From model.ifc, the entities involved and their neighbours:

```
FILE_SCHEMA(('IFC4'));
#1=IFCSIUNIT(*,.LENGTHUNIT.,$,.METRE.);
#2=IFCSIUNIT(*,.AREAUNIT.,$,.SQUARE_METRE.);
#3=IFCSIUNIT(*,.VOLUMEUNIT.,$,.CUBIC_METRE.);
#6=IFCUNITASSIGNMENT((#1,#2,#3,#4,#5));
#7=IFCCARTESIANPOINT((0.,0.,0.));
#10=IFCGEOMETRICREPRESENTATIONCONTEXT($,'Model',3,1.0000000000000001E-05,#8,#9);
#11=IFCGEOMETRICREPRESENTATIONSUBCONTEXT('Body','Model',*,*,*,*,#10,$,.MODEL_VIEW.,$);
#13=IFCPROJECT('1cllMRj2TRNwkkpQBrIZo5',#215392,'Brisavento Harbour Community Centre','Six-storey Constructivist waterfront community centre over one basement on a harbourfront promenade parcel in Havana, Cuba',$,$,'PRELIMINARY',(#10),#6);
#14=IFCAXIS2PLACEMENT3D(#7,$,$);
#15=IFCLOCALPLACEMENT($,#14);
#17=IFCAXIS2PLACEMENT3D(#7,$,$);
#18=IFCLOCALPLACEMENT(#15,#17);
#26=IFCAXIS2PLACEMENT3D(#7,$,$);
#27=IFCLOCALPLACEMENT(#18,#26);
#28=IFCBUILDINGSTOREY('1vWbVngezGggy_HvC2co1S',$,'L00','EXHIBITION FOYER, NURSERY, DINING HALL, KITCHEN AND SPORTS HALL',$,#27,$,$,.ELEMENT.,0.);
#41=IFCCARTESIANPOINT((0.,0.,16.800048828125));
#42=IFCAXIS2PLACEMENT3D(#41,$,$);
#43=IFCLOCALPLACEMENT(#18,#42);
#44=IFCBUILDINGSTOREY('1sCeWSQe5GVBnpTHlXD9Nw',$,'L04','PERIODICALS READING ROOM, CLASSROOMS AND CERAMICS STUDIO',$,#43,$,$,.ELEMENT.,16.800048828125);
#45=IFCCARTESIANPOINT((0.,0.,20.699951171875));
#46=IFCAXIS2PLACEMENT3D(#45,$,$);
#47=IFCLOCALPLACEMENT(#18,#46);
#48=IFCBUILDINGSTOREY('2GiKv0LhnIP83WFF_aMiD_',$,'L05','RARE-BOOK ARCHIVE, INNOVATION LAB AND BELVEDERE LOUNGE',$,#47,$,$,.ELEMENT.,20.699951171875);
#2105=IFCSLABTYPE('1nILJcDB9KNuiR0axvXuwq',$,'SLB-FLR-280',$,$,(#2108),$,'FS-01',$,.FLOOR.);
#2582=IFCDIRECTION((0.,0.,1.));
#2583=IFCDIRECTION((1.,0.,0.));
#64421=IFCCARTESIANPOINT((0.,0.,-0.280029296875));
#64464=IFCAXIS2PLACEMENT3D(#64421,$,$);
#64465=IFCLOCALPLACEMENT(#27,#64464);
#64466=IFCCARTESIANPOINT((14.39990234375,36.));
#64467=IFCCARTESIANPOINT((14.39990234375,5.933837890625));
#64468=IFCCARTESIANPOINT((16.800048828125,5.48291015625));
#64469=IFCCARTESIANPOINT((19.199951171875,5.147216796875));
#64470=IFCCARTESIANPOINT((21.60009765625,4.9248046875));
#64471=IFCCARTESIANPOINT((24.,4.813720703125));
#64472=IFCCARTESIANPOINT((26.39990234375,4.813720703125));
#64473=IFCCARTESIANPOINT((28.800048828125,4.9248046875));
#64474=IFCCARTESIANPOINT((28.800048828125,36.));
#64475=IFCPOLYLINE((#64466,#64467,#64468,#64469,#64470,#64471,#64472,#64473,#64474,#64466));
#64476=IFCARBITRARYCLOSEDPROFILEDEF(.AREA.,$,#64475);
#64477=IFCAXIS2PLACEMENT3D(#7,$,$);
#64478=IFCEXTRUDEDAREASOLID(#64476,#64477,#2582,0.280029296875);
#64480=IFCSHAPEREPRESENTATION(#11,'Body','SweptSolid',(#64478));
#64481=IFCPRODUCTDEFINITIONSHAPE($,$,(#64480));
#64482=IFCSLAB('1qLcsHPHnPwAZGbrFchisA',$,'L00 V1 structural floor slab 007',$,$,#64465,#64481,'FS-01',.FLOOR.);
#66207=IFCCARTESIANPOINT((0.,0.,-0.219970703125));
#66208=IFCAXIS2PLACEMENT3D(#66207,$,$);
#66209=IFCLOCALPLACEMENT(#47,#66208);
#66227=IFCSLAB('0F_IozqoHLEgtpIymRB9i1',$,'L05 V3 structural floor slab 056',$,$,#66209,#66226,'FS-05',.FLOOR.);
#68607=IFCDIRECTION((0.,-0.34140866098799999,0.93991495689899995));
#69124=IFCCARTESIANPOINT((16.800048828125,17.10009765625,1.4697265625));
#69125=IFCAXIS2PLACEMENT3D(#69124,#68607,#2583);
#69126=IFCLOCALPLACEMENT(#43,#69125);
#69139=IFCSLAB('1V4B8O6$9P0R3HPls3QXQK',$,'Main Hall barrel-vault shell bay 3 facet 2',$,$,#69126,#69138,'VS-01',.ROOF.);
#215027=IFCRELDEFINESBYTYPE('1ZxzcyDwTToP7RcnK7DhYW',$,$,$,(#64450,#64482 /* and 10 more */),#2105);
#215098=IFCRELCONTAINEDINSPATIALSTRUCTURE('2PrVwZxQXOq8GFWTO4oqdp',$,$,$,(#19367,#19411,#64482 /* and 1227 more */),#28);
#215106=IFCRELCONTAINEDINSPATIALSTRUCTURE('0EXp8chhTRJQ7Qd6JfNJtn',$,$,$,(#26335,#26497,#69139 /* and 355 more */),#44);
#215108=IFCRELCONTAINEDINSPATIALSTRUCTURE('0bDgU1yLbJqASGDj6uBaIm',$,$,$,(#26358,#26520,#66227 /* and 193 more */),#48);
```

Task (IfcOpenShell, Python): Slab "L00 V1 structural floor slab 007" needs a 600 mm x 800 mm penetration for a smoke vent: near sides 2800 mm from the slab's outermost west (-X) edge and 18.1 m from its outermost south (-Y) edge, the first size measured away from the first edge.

```python
import numpy as np
import ifcopenshell
import ifcopenshell.api.feature
import ifcopenshell.api.geometry
import ifcopenshell.api.root
import ifcopenshell.geom
import ifcopenshell.util.placement
import ifcopenshell.util.representation
import ifcopenshell.util.shape
import ifcopenshell.util.unit

model = ifcopenshell.open("model.ifc")
unit_scale = ifcopenshell.util.unit.calculate_unit_scale(model)
settings = ifcopenshell.geom.settings()


def volume(element):
    """Net volume in cubic metres, openings subtracted."""
    shape = ifcopenshell.geom.create_shape(settings, element)
    return ifcopenshell.util.shape.get_volume(shape.geometry)


slab = model.by_guid("1qLcsHPHnPwAZGbrFchisA")
before = volume(slab)

# Extent in the slab's own axes, in metres. The edges named are its -X and -Y sides.
slab_shape = ifcopenshell.geom.create_shape(settings, slab)
vertices = ifcopenshell.util.shape.get_vertices(slab_shape.geometry)
x_min, y_min, bottom = vertices.min(axis=0)
top = vertices[:, 2].max()

opening = ifcopenshell.api.root.create_entity(model, ifc_class="IfcOpeningElement", name="Smoke vent opening", predefined_type="OPENING")
context = ifcopenshell.util.representation.get_context(model, "Model", "Body", "MODEL_VIEW")
width, depth = 0.6, 0.8
outline = [(0.0, 0.0), (width, 0.0), (width, depth), (0.0, depth), (0.0, 0.0)]
# Overshoot both faces by 50 mm so the cut is clean.
shape = ifcopenshell.api.geometry.add_slab_representation(
    model, context=context, depth=top - bottom + 0.1, polyline=outline
)
ifcopenshell.api.geometry.assign_representation(model, product=opening, representation=shape)

matrix = ifcopenshell.util.placement.get_local_placement(slab.ObjectPlacement)
matrix[:, 3] = matrix @ np.append(np.array([x_min + 2.8, y_min + 18.1, bottom - 0.05]) / unit_scale, 1.0)
ifcopenshell.api.geometry.edit_object_placement(model, product=opening, matrix=matrix, is_si=False)
ifcopenshell.api.feature.add_feature(model, feature=opening, element=slab)

after = volume(slab)

print(f"slab volume {before:.3f} -> {after:.3f} m3")

model.write("model_updated.ifc")
```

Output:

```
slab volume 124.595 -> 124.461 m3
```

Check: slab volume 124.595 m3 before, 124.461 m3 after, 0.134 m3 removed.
